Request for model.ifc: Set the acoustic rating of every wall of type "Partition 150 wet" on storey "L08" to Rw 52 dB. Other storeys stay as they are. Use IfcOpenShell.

First a look at what the model holds.

```python
import ifcopenshell
import ifcopenshell.util.element

model = ifcopenshell.open("model.ifc")
print(model.schema)
storey = next(s for s in model.by_type("IfcBuildingStorey") if s.Name == "L08")
walls = [e for e in ifcopenshell.util.element.get_decomposition(storey) if e.is_a("IfcWall")]
seen = {}
for e in walls:
    element_type = ifcopenshell.util.element.get_type(e)
    key = (element_type.Name if element_type != e and element_type else None, ifcopenshell.util.element.get_pset(e, "Pset_WallCommon", "AcousticRating"))
    seen[key] = seen.get(key, 0) + 1
for (name, value), count in sorted(seen.items(), key=str):
    print(count, "x", name, "|", value)
```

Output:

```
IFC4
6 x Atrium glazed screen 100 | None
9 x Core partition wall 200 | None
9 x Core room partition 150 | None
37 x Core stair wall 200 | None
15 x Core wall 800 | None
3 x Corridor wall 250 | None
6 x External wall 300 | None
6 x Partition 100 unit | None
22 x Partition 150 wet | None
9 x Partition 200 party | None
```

```python
import ifcopenshell
import ifcopenshell.api.pset
import ifcopenshell.util.element

model = ifcopenshell.open("model.ifc")

storey = next(s for s in model.by_type("IfcBuildingStorey") if s.Name == "L08")
walls = [e for e in ifcopenshell.util.element.get_decomposition(storey) if e.is_a("IfcWall")]

count = 0
for e in walls:
    element_type = ifcopenshell.util.element.get_type(e)
    if element_type in (None, e) or element_type.Name != "Partition 150 wet":
        continue
    found = ifcopenshell.util.element.get_pset(e, "Pset_WallCommon", should_inherit=False)
    if found:
        pset = model.by_id(found["id"])
        if len(ifcopenshell.util.element.get_elements_by_pset(pset)) > 1:
            pset = ifcopenshell.api.pset.unshare_pset(model, products=[e], pset=pset)[0]
    else:
        pset = ifcopenshell.api.pset.add_pset(model, product=e, name="Pset_WallCommon")
    ifcopenshell.api.pset.edit_pset(model, pset=pset, properties={"AcousticRating": "Rw 52 dB"})
    count += 1

print(count, "walls updated")

model.write("model_updated.ifc")
```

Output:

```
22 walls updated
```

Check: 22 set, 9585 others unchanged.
